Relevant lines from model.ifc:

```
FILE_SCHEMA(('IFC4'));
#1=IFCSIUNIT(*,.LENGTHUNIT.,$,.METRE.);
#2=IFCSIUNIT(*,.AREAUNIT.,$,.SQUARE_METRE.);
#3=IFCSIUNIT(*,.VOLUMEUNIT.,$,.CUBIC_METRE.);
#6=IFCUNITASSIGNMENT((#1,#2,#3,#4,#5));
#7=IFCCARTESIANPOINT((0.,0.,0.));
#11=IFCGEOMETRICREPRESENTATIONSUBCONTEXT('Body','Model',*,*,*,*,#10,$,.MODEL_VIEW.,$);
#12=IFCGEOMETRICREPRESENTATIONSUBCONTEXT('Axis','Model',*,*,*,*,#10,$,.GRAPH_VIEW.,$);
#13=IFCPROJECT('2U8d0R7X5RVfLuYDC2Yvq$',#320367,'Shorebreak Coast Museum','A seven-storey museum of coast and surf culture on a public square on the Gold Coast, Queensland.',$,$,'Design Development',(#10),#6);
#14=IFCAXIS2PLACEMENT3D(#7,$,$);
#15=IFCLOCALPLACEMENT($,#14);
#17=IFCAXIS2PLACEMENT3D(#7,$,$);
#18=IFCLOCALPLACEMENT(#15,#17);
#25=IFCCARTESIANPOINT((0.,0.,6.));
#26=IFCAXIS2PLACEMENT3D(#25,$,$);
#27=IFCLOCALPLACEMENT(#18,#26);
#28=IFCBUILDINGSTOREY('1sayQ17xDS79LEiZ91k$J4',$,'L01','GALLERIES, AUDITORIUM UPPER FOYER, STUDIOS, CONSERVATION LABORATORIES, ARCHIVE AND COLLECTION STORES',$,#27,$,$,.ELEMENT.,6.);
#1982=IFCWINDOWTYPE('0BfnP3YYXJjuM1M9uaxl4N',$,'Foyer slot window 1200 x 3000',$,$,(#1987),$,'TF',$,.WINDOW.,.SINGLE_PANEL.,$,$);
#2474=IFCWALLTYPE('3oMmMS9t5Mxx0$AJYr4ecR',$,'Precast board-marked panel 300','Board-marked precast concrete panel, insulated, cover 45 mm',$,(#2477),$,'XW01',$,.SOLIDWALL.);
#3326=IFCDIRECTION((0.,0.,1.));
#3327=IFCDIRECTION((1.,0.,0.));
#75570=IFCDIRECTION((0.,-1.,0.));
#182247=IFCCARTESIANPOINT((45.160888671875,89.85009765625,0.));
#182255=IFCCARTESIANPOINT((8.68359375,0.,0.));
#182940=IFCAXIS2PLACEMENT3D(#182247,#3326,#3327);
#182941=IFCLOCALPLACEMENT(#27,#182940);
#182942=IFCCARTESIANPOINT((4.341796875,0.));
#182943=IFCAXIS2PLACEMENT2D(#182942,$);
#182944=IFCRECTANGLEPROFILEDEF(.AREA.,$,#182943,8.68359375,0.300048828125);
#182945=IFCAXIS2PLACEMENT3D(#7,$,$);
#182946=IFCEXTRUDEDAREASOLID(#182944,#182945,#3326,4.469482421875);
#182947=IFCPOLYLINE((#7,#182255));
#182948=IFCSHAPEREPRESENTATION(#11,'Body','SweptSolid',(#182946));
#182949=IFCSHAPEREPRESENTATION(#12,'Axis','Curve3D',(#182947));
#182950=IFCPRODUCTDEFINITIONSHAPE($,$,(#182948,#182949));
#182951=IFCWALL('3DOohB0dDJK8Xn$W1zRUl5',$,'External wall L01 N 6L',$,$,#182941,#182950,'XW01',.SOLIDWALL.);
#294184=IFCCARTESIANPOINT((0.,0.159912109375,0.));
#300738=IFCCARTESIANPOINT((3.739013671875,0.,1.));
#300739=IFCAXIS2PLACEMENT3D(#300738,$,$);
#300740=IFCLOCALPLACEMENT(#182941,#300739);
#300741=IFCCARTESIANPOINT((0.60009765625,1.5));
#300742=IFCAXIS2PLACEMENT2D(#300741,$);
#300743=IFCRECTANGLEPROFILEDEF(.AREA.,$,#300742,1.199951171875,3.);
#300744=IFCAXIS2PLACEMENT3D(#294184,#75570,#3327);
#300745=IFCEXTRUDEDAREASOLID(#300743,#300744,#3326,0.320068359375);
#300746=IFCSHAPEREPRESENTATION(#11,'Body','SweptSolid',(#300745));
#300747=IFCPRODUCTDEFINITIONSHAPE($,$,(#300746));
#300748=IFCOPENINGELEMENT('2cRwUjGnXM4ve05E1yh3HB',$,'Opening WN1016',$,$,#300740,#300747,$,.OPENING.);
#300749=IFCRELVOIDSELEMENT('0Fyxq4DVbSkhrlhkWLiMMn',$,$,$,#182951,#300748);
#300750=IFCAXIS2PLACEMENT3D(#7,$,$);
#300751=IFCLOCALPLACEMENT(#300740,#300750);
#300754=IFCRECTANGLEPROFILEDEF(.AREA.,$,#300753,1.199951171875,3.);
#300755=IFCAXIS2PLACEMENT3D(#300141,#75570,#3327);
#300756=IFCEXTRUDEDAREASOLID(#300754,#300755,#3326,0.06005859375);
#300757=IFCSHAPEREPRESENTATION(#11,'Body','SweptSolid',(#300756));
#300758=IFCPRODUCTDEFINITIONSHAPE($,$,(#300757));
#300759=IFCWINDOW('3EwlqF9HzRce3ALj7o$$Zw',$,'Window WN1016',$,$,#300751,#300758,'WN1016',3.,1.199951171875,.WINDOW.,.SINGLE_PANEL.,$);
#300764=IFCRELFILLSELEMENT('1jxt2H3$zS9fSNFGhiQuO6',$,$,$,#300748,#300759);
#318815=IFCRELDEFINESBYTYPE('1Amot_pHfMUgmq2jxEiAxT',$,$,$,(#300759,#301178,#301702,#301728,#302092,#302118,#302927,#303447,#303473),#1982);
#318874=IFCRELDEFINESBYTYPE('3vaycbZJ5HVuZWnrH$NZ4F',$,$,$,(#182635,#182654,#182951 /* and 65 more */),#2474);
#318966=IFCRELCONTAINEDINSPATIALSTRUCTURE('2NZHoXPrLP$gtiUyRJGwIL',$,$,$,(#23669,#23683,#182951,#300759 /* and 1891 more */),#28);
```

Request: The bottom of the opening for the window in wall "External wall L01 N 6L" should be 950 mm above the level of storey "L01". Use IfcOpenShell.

```python
import numpy as np
import ifcopenshell
import ifcopenshell.api.geometry
import ifcopenshell.geom
import ifcopenshell.util.element
import ifcopenshell.util.placement
import ifcopenshell.util.shape
import ifcopenshell.util.unit

model = ifcopenshell.open("model.ifc")
unit_scale = ifcopenshell.util.unit.calculate_unit_scale(model)

window = model.by_id(300759)
opening = window.FillsVoids[0].RelatingOpeningElement
storey = ifcopenshell.util.element.get_container(window, ifc_class="IfcBuildingStorey")
level = ifcopenshell.util.placement.get_local_placement(storey.ObjectPlacement)[2, 3]

# The opening's origin need not be at the sill, so measure its lowest point.
shape = ifcopenshell.geom.create_shape(ifcopenshell.geom.settings(), opening)
bottom = ifcopenshell.util.shape.get_shape_bottom_elevation(shape, shape.geometry) / unit_scale
dz = level + 0.95 / unit_scale - bottom

shift = np.array([0.0, 0.0, dz])
# The window is placed relative to its opening, so it follows when the opening moves.
matrix = ifcopenshell.util.placement.get_local_placement(opening.ObjectPlacement)
matrix[:3, 3] += shift
ifcopenshell.api.geometry.edit_object_placement(
    model, product=opening, matrix=matrix, is_si=False, should_transform_children=True
)

print(f"moved by {dz * unit_scale:+.3f} m")

model.write("model_v2.ifc")
```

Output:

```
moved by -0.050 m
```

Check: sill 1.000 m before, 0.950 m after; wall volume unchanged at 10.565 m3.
